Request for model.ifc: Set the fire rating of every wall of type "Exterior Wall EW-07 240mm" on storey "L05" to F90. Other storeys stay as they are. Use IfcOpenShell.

First a look at what the model holds.

```python
import ifcopenshell
import ifcopenshell.util.element

model = ifcopenshell.open("model.ifc")
print(model.schema)
storey = next(s for s in model.by_type("IfcBuildingStorey") if s.Name == "L05")
walls = [e for e in ifcopenshell.util.element.get_decomposition(storey) if e.is_a("IfcWall")]
seen = {}
for e in walls:
    element_type = ifcopenshell.util.element.get_type(e)
    key = (element_type.Name if element_type != e and element_type else None, ifcopenshell.util.element.get_pset(e, "Pset_WallCommon", "FireRating"))
    seen[key] = seen.get(key, 0) + 1
for (name, value), count in sorted(seen.items(), key=str):
    print(count, "x", name, "|", value)
```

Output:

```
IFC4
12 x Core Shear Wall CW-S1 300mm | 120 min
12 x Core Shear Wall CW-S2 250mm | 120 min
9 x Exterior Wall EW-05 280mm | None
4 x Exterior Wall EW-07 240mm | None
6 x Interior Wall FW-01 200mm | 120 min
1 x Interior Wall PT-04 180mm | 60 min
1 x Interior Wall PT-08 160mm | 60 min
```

```python
import ifcopenshell
import ifcopenshell.api.pset
import ifcopenshell.util.element

model = ifcopenshell.open("model.ifc")

storey = next(s for s in model.by_type("IfcBuildingStorey") if s.Name == "L05")
walls = [e for e in ifcopenshell.util.element.get_decomposition(storey) if e.is_a("IfcWall")]

count = 0
for e in walls:
    element_type = ifcopenshell.util.element.get_type(e)
    if element_type in (None, e) or element_type.Name != "Exterior Wall EW-07 240mm":
        continue
    # add_pset returns the element's existing set when there is one.
    pset = ifcopenshell.api.pset.add_pset(model, product=e, name="Pset_WallCommon")
    ifcopenshell.api.pset.edit_pset(model, pset=pset, properties={"FireRating": "F90"})
    count += 1

print(count, "walls updated")

model.write("model_edited.ifc")
```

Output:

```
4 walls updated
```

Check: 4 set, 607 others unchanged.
